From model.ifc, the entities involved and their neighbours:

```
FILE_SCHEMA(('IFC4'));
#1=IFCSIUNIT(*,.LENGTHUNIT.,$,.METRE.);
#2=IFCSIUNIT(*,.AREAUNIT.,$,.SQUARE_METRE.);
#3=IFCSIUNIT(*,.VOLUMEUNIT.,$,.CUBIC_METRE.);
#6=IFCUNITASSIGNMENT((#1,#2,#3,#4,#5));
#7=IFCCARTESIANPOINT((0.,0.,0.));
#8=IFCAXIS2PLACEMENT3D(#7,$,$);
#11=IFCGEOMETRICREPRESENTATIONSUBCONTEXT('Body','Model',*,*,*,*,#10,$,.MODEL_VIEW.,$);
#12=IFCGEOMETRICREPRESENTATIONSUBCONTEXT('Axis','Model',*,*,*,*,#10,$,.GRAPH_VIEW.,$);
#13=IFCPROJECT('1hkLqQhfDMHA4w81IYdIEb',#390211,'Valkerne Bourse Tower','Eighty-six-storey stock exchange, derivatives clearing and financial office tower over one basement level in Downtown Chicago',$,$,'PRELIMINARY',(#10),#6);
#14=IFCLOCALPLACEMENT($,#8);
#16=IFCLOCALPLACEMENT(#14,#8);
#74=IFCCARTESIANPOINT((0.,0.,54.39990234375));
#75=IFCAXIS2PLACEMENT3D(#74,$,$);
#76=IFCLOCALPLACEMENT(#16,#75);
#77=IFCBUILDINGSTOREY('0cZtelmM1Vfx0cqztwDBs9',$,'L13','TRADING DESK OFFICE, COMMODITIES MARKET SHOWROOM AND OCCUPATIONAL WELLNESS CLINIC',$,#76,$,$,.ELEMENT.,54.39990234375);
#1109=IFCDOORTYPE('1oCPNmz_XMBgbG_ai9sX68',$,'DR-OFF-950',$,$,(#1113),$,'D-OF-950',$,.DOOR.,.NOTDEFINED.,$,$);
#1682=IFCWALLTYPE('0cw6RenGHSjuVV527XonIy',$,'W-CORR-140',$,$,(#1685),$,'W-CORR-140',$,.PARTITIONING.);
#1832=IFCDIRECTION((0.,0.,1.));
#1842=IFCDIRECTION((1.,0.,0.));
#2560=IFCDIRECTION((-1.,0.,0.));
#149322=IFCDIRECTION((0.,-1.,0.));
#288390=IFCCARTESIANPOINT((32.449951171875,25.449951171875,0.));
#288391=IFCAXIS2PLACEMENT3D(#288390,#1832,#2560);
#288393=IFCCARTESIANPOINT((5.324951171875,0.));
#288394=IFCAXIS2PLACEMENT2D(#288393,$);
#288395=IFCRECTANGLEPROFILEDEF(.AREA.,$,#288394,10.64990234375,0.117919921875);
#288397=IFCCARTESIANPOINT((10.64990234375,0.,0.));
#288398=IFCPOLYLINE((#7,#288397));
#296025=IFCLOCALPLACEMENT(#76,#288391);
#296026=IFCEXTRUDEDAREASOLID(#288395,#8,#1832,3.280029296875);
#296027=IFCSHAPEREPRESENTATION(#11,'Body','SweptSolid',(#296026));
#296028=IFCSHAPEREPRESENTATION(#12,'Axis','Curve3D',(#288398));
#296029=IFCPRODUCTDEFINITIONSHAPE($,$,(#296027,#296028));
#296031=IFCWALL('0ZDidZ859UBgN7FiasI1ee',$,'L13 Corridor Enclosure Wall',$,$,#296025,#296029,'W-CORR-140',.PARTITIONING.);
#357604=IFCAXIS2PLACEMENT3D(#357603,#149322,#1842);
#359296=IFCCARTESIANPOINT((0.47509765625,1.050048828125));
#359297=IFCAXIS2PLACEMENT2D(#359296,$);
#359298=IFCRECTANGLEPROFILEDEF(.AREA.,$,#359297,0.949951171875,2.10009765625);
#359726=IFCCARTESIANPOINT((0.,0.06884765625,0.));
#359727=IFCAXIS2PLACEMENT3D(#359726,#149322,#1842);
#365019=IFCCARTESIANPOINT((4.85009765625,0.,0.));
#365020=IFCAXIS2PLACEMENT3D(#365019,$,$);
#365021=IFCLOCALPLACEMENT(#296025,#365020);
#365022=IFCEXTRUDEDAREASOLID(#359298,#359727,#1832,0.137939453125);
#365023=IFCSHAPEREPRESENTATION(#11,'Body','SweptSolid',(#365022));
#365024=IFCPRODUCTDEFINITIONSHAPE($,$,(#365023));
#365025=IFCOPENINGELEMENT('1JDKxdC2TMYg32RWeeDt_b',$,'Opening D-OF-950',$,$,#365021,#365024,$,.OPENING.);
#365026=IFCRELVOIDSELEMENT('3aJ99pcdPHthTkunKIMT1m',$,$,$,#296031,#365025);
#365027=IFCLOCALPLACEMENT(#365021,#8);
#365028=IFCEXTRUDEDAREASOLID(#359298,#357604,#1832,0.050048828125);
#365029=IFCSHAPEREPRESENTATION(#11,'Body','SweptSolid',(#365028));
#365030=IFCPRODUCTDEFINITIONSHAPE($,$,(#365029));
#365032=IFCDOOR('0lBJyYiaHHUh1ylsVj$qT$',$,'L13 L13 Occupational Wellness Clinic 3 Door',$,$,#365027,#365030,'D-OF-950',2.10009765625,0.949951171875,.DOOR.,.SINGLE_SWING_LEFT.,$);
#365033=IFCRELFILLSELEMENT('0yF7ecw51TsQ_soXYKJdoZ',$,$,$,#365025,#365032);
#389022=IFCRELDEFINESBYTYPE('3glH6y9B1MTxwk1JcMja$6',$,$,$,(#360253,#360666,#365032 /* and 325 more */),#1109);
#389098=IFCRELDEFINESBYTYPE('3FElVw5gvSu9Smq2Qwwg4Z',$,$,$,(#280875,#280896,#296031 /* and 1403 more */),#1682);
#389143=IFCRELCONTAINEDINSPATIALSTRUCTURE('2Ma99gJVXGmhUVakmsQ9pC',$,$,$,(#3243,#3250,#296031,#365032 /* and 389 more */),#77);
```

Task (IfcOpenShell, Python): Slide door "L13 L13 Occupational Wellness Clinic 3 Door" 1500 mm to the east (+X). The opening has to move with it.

```python
import ifcopenshell
import ifcopenshell.api.geometry
import ifcopenshell.util.placement
import ifcopenshell.util.unit

model = ifcopenshell.open("model.ifc")
unit_scale = ifcopenshell.util.unit.calculate_unit_scale(model)

door = model.by_guid("0lBJyYiaHHUh1ylsVj$qT$")
opening = door.FillsVoids[0].RelatingOpeningElement
wall = opening.VoidsElements[0].RelatingBuildingElement

wall_matrix = ifcopenshell.util.placement.get_local_placement(wall.ObjectPlacement)
shift = wall_matrix[:3, 0] * -1.5 / unit_scale
before = ifcopenshell.util.placement.get_local_placement(door.ObjectPlacement)[:3, 3].copy()

# The door is placed relative to its opening, so it follows when the opening moves.
matrix = ifcopenshell.util.placement.get_local_placement(opening.ObjectPlacement)
matrix[:3, 3] += shift
ifcopenshell.api.geometry.edit_object_placement(
    model, product=opening, matrix=matrix, is_si=False, should_transform_children=True
)

after = ifcopenshell.util.placement.get_local_placement(door.ObjectPlacement)[:3, 3]
print("door moved by", (after - before).round(3) + 0.0)

model.write("model_rev.ifc")
```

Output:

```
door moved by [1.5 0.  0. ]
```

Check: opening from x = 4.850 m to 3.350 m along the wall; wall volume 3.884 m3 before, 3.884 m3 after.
